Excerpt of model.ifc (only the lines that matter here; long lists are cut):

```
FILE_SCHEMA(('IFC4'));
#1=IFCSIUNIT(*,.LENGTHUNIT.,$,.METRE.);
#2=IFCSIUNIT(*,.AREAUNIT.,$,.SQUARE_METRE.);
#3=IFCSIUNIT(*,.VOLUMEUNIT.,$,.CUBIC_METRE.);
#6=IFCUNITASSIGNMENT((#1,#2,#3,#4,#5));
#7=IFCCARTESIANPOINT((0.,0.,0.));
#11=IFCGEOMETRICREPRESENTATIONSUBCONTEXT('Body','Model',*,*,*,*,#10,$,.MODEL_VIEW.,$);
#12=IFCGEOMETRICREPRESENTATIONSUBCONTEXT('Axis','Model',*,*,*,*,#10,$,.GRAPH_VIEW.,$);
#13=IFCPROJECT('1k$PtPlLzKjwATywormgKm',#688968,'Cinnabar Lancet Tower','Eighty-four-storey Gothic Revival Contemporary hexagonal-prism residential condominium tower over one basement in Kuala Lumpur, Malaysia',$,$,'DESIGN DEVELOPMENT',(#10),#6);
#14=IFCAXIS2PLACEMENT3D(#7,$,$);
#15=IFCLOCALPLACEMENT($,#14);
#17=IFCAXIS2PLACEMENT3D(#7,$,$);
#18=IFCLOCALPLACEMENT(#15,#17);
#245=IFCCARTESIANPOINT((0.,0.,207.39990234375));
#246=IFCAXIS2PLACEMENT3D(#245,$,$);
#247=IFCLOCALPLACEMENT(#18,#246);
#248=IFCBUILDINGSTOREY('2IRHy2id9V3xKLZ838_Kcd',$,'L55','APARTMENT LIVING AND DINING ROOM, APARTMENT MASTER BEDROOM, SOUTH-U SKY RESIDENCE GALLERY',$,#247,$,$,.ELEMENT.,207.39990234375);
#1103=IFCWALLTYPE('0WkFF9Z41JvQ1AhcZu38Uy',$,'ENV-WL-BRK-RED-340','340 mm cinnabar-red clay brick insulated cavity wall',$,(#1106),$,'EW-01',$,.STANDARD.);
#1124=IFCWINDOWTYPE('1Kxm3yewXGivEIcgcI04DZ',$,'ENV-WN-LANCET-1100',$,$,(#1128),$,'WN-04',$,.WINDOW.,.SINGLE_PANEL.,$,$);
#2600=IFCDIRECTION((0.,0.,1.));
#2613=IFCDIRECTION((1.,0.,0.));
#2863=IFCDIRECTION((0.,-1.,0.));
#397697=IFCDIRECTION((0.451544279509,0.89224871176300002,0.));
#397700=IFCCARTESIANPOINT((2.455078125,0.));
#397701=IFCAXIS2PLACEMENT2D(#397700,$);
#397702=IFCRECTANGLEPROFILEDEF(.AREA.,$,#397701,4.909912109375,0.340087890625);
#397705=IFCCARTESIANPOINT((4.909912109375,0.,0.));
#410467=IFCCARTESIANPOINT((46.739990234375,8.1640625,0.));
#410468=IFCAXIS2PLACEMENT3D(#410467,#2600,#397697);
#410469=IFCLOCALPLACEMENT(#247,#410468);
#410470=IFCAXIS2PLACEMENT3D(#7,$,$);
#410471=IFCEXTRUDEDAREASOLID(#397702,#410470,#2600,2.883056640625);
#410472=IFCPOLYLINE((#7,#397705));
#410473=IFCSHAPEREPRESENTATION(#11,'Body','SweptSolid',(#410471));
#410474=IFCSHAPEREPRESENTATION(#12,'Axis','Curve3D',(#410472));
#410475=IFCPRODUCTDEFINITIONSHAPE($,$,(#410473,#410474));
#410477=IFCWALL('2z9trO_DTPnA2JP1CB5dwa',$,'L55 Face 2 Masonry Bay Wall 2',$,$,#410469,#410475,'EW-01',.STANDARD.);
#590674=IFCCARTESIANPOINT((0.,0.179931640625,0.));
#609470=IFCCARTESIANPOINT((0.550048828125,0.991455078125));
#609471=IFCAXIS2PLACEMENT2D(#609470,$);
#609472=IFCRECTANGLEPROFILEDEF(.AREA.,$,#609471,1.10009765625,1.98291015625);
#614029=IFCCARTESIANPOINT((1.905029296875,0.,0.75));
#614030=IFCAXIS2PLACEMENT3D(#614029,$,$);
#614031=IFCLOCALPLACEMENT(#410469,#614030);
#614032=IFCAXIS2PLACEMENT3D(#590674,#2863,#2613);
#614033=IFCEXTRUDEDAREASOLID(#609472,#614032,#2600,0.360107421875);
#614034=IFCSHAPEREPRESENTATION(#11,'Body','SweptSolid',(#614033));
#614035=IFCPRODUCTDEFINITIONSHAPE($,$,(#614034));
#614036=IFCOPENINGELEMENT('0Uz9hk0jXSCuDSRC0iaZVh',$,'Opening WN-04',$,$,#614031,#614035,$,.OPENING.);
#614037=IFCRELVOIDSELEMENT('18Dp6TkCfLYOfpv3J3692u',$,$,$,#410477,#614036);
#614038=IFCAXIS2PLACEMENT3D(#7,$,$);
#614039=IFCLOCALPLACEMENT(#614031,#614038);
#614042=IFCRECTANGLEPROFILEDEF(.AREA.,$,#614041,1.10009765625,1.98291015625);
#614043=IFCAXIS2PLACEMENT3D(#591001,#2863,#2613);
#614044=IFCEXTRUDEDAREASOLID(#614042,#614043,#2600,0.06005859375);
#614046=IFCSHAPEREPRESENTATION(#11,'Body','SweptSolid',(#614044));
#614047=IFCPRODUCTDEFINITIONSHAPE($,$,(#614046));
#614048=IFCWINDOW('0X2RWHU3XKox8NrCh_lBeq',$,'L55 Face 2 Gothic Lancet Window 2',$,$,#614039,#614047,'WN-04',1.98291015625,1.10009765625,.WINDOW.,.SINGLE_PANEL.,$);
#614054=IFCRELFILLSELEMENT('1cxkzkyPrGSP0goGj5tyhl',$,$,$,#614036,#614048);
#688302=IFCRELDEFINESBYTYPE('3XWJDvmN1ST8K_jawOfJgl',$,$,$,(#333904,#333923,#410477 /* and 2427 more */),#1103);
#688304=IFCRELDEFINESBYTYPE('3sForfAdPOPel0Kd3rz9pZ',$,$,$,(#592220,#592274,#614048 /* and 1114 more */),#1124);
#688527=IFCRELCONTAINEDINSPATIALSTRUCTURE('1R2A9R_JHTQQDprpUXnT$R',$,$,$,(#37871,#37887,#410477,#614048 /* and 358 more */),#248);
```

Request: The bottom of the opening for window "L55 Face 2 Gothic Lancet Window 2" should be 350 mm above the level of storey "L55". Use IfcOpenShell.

```python
import numpy as np
import ifcopenshell
import ifcopenshell.api.geometry
import ifcopenshell.geom
import ifcopenshell.util.element
import ifcopenshell.util.placement
import ifcopenshell.util.shape
import ifcopenshell.util.unit

model = ifcopenshell.open("model.ifc")
unit_scale = ifcopenshell.util.unit.calculate_unit_scale(model)

window = model.by_guid("0X2RWHU3XKox8NrCh_lBeq")
opening = window.FillsVoids[0].RelatingOpeningElement
storey = ifcopenshell.util.element.get_container(window, ifc_class="IfcBuildingStorey")
level = ifcopenshell.util.placement.get_local_placement(storey.ObjectPlacement)[2, 3]

# The opening's origin need not be at the sill, so measure its lowest point.
shape = ifcopenshell.geom.create_shape(ifcopenshell.geom.settings(), opening)
bottom = ifcopenshell.util.shape.get_shape_bottom_elevation(shape, shape.geometry) / unit_scale
dz = level + 0.35 / unit_scale - bottom

shift = np.array([0.0, 0.0, dz])
# The window is placed relative to its opening, so it follows when the opening moves.
matrix = ifcopenshell.util.placement.get_local_placement(opening.ObjectPlacement)
matrix[:3, 3] += shift
ifcopenshell.api.geometry.edit_object_placement(
    model, product=opening, matrix=matrix, is_si=False, should_transform_children=True
)

print(f"moved by {dz * unit_scale:+.3f} m")

model.write("model-out.ifc")
```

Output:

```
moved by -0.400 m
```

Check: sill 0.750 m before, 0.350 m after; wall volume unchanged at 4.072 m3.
